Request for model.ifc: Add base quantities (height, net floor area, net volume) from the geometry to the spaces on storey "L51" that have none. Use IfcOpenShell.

First a look at what the model holds.

```python
import ifcopenshell
import ifcopenshell.util.element
import ifcopenshell.util.unit

model = ifcopenshell.open("model.ifc")
print(model.schema)
for unit_type in ("LENGTHUNIT", "AREAUNIT", "VOLUMEUNIT"):
    print(unit_type, ifcopenshell.util.unit.calculate_unit_scale(model, unit_type))
storey = next(s for s in model.by_type("IfcBuildingStorey") if s.Name == "L51")
spaces = [e for e in ifcopenshell.util.element.get_decomposition(storey) if e.is_a("IfcSpace")]
for e in sorted(spaces, key=lambda e: e.id()):
    print(e.id(), e.is_a(), e.Name, list(ifcopenshell.util.element.get_psets(e, qtos_only=True)), sep=" | ")
```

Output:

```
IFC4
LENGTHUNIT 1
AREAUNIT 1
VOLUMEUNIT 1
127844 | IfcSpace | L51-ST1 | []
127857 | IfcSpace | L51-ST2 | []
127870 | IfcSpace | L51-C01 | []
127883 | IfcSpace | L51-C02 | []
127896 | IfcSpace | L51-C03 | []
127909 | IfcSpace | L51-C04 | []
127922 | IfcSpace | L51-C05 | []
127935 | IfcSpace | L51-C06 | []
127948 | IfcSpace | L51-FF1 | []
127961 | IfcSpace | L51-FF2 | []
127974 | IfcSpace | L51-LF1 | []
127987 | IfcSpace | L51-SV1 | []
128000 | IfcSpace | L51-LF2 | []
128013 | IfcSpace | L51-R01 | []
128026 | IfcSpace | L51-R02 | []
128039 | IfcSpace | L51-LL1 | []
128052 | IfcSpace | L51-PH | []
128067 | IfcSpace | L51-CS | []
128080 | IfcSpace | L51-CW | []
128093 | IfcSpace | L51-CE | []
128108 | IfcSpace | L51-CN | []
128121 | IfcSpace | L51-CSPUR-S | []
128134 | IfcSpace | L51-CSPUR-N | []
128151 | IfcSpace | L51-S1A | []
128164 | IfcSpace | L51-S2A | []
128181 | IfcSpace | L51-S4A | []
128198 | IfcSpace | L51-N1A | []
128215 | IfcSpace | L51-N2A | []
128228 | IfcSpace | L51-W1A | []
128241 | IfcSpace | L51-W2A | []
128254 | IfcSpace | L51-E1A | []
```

```python
import ifcopenshell
import ifcopenshell.api.pset
import ifcopenshell.geom
import ifcopenshell.util.element
import ifcopenshell.util.shape
import ifcopenshell.util.unit

model = ifcopenshell.open("model.ifc")
unit_scale = ifcopenshell.util.unit.calculate_unit_scale(model)
area_scale = ifcopenshell.util.unit.calculate_unit_scale(model, "AREAUNIT")
volume_scale = ifcopenshell.util.unit.calculate_unit_scale(model, "VOLUMEUNIT")
settings = ifcopenshell.geom.settings()

storey = next(s for s in model.by_type("IfcBuildingStorey") if s.Name == "L51")
spaces = [e for e in ifcopenshell.util.element.get_decomposition(storey) if e.is_a("IfcSpace")]

for e in sorted(spaces, key=lambda e: e.id()):
    if ifcopenshell.util.element.get_psets(e, qtos_only=True, should_inherit=False):
        continue
    # Geometry comes back in metres, in the element's own axes.
    shape = ifcopenshell.geom.create_shape(settings, e)
    values = {
        "Height": ifcopenshell.util.shape.get_z(shape.geometry) / unit_scale,
        "NetFloorArea": ifcopenshell.util.shape.get_footprint_area(shape.geometry) / area_scale,
        "NetVolume": ifcopenshell.util.shape.get_volume(shape.geometry) / volume_scale,
    }
    qto = ifcopenshell.api.pset.add_qto(model, product=e, name="Qto_SpaceBaseQuantities")
    ifcopenshell.api.pset.edit_qto(model, qto=qto, properties=values)
    print(e.id(), {k: round(v, 3) for k, v in values.items()})

model.write("model_rev.ifc")
```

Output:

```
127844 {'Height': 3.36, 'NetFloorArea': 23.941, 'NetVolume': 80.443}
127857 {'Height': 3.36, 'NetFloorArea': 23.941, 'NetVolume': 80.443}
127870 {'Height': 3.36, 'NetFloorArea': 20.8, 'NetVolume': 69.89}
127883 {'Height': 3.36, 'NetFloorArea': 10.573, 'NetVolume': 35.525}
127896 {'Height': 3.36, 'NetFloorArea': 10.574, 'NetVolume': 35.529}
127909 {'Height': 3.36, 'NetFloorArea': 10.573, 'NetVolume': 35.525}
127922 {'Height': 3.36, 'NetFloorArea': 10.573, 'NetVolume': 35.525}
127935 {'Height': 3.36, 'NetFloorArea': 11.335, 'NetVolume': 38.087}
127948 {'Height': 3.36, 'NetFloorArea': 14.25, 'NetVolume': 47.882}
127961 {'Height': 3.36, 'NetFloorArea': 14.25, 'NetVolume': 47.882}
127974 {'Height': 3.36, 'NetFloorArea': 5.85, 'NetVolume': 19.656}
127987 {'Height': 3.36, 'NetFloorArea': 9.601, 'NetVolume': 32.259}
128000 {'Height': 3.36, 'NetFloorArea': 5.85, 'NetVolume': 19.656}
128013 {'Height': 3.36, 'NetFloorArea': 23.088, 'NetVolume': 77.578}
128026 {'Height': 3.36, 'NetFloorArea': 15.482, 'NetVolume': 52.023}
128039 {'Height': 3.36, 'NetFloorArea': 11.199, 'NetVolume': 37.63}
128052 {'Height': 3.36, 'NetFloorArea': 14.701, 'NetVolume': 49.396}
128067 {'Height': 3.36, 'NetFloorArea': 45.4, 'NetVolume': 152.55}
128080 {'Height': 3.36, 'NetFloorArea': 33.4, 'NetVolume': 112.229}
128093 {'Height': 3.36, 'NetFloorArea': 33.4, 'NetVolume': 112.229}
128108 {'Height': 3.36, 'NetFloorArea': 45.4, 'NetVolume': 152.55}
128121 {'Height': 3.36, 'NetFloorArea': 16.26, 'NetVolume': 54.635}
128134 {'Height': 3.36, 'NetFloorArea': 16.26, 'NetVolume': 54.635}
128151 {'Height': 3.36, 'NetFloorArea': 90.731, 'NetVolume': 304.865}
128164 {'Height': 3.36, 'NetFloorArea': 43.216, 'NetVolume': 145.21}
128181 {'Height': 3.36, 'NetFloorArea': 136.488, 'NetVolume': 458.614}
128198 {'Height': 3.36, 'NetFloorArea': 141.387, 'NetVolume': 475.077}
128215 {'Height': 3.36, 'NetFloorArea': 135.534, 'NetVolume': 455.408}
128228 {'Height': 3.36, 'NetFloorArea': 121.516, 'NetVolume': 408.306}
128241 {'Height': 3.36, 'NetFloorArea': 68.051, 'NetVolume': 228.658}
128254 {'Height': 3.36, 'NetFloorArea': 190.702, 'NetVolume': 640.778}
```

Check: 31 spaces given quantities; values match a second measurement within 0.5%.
